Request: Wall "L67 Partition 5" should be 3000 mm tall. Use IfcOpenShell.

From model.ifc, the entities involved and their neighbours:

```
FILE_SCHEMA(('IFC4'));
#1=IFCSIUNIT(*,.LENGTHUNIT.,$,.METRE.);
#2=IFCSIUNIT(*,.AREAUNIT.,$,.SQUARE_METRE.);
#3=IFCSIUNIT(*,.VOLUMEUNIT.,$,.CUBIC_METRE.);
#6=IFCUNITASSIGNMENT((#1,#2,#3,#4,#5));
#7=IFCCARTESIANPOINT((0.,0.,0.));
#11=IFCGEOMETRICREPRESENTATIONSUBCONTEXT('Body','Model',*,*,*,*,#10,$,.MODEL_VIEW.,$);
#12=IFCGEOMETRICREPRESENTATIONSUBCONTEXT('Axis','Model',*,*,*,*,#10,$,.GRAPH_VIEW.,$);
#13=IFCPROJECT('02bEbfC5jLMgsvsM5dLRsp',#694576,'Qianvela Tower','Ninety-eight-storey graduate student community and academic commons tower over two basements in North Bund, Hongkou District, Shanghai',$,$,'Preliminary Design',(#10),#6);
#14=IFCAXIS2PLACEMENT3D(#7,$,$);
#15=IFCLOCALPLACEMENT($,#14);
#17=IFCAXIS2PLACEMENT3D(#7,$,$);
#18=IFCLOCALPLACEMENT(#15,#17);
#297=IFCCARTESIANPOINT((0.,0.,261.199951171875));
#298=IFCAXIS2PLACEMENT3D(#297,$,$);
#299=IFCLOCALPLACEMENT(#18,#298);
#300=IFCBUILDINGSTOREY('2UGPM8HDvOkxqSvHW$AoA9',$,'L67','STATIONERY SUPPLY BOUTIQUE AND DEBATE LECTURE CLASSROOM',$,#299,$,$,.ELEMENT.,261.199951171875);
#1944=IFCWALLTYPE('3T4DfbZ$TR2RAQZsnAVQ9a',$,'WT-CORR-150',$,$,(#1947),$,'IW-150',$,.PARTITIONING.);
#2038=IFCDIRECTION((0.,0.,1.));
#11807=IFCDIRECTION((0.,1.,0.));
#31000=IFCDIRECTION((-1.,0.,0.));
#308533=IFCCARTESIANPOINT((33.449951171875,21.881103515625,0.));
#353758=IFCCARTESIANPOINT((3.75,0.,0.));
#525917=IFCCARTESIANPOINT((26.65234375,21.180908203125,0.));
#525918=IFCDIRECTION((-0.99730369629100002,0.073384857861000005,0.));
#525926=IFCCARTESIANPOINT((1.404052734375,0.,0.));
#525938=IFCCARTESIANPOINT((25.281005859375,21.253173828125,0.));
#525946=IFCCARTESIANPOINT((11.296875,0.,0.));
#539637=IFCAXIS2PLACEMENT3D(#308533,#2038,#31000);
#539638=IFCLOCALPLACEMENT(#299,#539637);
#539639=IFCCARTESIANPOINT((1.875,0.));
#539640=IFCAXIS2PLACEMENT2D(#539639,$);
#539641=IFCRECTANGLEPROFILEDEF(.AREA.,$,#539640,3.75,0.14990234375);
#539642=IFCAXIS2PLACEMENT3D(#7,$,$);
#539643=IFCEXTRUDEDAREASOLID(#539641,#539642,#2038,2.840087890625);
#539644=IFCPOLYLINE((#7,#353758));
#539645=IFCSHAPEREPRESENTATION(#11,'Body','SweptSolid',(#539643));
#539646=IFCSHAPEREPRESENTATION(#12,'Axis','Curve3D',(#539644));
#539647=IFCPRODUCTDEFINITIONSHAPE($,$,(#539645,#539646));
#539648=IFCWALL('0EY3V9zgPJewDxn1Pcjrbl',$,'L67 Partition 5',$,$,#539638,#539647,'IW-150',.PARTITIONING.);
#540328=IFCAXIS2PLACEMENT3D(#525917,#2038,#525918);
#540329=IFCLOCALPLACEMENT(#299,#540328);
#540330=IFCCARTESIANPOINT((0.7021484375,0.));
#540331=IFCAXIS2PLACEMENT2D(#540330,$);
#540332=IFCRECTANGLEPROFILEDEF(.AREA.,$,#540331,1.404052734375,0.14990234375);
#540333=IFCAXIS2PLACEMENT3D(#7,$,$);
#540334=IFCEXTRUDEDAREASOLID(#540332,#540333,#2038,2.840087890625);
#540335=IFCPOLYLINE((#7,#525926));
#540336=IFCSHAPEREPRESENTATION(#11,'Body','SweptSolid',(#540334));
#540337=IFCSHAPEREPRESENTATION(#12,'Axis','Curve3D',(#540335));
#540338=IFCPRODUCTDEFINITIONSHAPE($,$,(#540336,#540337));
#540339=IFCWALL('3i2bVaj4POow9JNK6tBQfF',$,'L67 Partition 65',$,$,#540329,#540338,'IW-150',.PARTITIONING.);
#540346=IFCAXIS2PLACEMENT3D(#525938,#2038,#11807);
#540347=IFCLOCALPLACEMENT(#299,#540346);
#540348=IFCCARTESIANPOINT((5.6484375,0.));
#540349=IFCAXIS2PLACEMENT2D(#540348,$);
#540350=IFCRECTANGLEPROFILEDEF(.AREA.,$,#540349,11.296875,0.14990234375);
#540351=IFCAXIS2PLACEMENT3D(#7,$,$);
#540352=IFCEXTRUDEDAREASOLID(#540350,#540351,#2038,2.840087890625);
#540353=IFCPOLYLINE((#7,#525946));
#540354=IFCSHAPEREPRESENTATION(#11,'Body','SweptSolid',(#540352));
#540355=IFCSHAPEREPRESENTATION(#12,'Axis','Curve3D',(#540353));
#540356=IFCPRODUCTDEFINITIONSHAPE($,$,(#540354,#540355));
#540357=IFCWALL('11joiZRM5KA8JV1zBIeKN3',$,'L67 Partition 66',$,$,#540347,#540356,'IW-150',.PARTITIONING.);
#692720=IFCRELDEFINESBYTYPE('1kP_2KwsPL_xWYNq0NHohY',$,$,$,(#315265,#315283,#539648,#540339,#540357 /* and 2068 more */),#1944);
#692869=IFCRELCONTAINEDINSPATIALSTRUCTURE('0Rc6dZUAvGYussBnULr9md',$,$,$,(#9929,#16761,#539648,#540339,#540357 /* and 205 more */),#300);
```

```python
import ifcopenshell
import ifcopenshell.geom
import ifcopenshell.util.representation
import ifcopenshell.util.shape
import ifcopenshell.util.unit

model = ifcopenshell.open("model.ifc")
unit_scale = ifcopenshell.util.unit.calculate_unit_scale(model)
settings = ifcopenshell.geom.settings()


def volume(element):
    """Net volume in cubic metres, openings subtracted."""
    shape = ifcopenshell.geom.create_shape(settings, element)
    return ifcopenshell.util.shape.get_volume(shape.geometry)


wall = model.by_guid("0EY3V9zgPJewDxn1Pcjrbl")
before = volume(wall)

body = ifcopenshell.util.representation.get_representation(wall, "Model", "Body")
solid = body.Items[0]
old_height = solid.Depth
solid.Depth = 3 / unit_scale
after = volume(wall)

print(f"height {old_height:g} -> {solid.Depth:g}, volume {before:.3f} -> {after:.3f} m3")

model.write("model_edited.ifc")
```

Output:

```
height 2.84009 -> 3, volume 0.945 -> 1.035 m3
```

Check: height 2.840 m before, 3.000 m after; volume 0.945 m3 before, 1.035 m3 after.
